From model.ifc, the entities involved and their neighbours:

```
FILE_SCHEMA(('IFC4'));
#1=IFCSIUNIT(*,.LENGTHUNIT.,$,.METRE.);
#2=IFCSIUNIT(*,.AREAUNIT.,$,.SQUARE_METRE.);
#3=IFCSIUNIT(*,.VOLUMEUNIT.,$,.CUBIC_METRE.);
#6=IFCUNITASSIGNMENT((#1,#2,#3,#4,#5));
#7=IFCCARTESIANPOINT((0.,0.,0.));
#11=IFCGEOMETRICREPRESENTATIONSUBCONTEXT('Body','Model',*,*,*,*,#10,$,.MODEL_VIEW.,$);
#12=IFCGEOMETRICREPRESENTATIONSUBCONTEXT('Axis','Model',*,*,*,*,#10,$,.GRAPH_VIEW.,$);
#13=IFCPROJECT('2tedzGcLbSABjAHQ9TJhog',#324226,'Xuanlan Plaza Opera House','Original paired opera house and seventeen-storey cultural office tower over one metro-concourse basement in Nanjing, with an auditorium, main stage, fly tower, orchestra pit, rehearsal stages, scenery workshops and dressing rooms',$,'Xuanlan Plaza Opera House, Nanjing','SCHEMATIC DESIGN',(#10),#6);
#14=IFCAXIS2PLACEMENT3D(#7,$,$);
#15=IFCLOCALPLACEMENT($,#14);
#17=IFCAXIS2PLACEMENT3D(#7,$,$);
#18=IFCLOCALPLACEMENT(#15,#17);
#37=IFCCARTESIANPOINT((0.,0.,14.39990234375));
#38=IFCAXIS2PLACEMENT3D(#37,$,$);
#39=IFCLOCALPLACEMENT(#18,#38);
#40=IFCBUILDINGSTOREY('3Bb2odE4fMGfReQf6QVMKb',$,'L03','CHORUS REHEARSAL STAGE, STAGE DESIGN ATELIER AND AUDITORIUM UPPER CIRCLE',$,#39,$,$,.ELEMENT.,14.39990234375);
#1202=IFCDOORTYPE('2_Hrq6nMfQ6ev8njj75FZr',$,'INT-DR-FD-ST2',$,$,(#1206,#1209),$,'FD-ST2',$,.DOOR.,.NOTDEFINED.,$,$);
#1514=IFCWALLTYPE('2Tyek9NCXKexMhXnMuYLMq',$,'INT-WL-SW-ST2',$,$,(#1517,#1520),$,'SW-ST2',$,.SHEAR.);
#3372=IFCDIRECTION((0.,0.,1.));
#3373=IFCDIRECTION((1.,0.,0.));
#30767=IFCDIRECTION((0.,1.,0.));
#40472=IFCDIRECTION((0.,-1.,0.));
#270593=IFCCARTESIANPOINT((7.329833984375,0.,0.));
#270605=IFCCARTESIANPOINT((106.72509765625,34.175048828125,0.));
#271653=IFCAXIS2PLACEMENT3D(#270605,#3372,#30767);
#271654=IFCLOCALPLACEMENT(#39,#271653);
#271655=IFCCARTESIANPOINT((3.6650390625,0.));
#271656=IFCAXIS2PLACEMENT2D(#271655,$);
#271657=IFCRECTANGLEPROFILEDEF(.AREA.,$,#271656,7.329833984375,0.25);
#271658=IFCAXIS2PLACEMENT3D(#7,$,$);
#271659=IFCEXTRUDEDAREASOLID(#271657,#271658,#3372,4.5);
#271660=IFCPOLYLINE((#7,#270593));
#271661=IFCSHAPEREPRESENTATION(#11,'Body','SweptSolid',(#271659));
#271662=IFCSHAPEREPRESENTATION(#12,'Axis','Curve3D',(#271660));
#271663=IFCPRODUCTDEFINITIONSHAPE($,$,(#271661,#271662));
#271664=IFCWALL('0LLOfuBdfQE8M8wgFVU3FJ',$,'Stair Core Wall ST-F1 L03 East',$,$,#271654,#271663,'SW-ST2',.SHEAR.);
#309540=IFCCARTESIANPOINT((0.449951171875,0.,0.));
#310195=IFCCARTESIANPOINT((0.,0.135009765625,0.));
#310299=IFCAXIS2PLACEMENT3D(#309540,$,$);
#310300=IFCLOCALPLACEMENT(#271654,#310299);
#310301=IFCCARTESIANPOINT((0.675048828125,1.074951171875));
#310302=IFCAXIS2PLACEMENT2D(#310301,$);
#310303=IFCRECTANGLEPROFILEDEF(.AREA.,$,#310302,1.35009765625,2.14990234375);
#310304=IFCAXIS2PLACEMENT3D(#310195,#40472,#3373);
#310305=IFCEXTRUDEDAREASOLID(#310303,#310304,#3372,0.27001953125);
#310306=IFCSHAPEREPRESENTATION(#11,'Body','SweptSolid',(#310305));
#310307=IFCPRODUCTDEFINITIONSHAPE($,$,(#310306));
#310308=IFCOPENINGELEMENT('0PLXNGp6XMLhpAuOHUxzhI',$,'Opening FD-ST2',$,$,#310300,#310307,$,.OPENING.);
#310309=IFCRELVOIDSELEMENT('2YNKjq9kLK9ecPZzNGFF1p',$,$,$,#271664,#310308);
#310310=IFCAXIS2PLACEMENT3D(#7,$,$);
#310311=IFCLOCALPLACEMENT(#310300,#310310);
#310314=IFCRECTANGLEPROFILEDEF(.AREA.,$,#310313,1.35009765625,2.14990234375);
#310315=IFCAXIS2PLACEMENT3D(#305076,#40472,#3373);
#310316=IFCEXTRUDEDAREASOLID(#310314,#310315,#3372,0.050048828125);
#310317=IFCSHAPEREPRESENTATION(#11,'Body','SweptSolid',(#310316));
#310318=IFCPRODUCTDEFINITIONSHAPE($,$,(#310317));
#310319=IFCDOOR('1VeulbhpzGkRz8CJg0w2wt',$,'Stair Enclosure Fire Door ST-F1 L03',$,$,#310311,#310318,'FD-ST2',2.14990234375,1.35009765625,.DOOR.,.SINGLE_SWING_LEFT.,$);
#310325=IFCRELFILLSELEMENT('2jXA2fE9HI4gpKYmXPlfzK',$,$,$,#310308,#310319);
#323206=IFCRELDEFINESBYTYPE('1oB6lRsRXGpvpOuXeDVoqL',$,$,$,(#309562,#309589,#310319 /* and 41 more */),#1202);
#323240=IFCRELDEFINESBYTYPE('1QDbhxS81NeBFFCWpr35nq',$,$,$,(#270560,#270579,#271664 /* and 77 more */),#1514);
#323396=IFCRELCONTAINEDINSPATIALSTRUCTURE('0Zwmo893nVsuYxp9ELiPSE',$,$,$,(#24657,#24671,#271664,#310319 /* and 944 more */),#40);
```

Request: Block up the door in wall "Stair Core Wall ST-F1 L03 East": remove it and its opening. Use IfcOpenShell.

```python
import ifcopenshell
import ifcopenshell.api.feature
import ifcopenshell.api.root
import ifcopenshell.geom
import ifcopenshell.util.shape

model = ifcopenshell.open("model.ifc")
settings = ifcopenshell.geom.settings()


def volume(element):
    """Net volume in cubic metres, openings subtracted."""
    shape = ifcopenshell.geom.create_shape(settings, element)
    return ifcopenshell.util.shape.get_volume(shape.geometry)


door = model.by_guid("1VeulbhpzGkRz8CJg0w2wt")
opening = door.FillsVoids[0].RelatingOpeningElement
wall = opening.VoidsElements[0].RelatingBuildingElement
before = volume(wall)

ifcopenshell.api.root.remove_product(model, product=door)
ifcopenshell.api.feature.remove_feature(model, feature=opening)

after = volume(wall)

print(f"wall volume {before:.3f} -> {after:.3f} m3")

model.write("model_updated.ifc")
```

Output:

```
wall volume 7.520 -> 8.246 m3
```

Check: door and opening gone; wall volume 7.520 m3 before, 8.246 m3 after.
